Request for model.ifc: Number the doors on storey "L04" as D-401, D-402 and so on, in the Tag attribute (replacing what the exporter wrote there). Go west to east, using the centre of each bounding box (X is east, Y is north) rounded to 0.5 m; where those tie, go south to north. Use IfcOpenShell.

First a look at what the model holds.

```python
import ifcopenshell
import ifcopenshell.util.element
import ifcopenshell.util.placement

model = ifcopenshell.open("model.ifc")
print(model.schema)
storey = next(s for s in model.by_type("IfcBuildingStorey") if s.Name == "L04")
doors = [e for e in ifcopenshell.util.element.get_decomposition(storey) if e.is_a("IfcDoor")]
for e in sorted(doors, key=lambda e: e.id()):
    origin = ifcopenshell.util.placement.get_local_placement(e.ObjectPlacement)[:3, 3]
    print(e.id(), e.Tag, e.Name, origin.round(2) + 0.0, sep=" | ")
```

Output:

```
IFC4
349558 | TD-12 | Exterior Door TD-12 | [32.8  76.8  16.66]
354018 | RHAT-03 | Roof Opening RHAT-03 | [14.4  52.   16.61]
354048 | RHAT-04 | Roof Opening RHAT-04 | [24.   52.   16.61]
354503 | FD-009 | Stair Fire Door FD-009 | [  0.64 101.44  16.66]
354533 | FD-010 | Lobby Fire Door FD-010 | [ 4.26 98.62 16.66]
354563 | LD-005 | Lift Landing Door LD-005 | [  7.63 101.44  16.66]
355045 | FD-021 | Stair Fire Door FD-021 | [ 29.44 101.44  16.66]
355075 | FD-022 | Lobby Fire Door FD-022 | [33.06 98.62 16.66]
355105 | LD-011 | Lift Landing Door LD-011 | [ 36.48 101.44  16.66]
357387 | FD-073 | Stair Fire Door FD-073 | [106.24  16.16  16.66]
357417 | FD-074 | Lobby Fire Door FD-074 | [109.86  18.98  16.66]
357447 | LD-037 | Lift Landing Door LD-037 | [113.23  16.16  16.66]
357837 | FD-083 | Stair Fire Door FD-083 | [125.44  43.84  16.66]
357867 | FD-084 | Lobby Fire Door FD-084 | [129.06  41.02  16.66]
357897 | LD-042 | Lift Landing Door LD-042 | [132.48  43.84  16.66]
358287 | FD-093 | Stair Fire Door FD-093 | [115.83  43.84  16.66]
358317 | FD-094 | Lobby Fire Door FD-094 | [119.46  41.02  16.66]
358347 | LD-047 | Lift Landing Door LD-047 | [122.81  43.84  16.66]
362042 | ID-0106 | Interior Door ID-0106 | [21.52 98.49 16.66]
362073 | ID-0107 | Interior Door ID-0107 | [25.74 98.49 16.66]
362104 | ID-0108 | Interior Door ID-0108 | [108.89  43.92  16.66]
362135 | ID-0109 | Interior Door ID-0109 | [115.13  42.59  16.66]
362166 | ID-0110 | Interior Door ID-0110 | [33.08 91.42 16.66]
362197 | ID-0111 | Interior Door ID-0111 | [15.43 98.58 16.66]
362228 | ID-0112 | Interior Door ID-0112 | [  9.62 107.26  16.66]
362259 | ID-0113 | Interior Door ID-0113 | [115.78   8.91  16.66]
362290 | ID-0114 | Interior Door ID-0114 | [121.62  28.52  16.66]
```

```python
import ifcopenshell
import ifcopenshell.geom
import ifcopenshell.util.element
import ifcopenshell.util.shape

model = ifcopenshell.open("model.ifc")
settings = ifcopenshell.geom.settings()
settings.set("use-world-coords", True)


def centre(element):
    shape = ifcopenshell.geom.create_shape(settings, element)
    return ifcopenshell.util.shape.get_bbox_centroid(shape.geometry)


storey = next(s for s in model.by_type("IfcBuildingStorey") if s.Name == "L04")
doors = [e for e in ifcopenshell.util.element.get_decomposition(storey) if e.is_a("IfcDoor")]

# Insertion points can sit at a corner or the storey origin, so sort by the geometry (in metres).
centres = {e: centre(e) for e in doors}
doors.sort(key=lambda e: (round(centres[e][0] / 0.5), centres[e][1]))

for i, e in enumerate(doors, start=1):
    number = f"D-4{i:02d}"
    e.Tag = number
    print(e.id(), number)

model.write("model_updated.ifc")
```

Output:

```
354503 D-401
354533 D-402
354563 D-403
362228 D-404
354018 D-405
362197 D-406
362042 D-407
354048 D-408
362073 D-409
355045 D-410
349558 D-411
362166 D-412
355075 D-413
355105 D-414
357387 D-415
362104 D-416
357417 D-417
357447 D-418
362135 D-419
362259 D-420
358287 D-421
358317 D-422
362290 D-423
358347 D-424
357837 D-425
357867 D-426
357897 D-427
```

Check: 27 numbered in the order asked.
